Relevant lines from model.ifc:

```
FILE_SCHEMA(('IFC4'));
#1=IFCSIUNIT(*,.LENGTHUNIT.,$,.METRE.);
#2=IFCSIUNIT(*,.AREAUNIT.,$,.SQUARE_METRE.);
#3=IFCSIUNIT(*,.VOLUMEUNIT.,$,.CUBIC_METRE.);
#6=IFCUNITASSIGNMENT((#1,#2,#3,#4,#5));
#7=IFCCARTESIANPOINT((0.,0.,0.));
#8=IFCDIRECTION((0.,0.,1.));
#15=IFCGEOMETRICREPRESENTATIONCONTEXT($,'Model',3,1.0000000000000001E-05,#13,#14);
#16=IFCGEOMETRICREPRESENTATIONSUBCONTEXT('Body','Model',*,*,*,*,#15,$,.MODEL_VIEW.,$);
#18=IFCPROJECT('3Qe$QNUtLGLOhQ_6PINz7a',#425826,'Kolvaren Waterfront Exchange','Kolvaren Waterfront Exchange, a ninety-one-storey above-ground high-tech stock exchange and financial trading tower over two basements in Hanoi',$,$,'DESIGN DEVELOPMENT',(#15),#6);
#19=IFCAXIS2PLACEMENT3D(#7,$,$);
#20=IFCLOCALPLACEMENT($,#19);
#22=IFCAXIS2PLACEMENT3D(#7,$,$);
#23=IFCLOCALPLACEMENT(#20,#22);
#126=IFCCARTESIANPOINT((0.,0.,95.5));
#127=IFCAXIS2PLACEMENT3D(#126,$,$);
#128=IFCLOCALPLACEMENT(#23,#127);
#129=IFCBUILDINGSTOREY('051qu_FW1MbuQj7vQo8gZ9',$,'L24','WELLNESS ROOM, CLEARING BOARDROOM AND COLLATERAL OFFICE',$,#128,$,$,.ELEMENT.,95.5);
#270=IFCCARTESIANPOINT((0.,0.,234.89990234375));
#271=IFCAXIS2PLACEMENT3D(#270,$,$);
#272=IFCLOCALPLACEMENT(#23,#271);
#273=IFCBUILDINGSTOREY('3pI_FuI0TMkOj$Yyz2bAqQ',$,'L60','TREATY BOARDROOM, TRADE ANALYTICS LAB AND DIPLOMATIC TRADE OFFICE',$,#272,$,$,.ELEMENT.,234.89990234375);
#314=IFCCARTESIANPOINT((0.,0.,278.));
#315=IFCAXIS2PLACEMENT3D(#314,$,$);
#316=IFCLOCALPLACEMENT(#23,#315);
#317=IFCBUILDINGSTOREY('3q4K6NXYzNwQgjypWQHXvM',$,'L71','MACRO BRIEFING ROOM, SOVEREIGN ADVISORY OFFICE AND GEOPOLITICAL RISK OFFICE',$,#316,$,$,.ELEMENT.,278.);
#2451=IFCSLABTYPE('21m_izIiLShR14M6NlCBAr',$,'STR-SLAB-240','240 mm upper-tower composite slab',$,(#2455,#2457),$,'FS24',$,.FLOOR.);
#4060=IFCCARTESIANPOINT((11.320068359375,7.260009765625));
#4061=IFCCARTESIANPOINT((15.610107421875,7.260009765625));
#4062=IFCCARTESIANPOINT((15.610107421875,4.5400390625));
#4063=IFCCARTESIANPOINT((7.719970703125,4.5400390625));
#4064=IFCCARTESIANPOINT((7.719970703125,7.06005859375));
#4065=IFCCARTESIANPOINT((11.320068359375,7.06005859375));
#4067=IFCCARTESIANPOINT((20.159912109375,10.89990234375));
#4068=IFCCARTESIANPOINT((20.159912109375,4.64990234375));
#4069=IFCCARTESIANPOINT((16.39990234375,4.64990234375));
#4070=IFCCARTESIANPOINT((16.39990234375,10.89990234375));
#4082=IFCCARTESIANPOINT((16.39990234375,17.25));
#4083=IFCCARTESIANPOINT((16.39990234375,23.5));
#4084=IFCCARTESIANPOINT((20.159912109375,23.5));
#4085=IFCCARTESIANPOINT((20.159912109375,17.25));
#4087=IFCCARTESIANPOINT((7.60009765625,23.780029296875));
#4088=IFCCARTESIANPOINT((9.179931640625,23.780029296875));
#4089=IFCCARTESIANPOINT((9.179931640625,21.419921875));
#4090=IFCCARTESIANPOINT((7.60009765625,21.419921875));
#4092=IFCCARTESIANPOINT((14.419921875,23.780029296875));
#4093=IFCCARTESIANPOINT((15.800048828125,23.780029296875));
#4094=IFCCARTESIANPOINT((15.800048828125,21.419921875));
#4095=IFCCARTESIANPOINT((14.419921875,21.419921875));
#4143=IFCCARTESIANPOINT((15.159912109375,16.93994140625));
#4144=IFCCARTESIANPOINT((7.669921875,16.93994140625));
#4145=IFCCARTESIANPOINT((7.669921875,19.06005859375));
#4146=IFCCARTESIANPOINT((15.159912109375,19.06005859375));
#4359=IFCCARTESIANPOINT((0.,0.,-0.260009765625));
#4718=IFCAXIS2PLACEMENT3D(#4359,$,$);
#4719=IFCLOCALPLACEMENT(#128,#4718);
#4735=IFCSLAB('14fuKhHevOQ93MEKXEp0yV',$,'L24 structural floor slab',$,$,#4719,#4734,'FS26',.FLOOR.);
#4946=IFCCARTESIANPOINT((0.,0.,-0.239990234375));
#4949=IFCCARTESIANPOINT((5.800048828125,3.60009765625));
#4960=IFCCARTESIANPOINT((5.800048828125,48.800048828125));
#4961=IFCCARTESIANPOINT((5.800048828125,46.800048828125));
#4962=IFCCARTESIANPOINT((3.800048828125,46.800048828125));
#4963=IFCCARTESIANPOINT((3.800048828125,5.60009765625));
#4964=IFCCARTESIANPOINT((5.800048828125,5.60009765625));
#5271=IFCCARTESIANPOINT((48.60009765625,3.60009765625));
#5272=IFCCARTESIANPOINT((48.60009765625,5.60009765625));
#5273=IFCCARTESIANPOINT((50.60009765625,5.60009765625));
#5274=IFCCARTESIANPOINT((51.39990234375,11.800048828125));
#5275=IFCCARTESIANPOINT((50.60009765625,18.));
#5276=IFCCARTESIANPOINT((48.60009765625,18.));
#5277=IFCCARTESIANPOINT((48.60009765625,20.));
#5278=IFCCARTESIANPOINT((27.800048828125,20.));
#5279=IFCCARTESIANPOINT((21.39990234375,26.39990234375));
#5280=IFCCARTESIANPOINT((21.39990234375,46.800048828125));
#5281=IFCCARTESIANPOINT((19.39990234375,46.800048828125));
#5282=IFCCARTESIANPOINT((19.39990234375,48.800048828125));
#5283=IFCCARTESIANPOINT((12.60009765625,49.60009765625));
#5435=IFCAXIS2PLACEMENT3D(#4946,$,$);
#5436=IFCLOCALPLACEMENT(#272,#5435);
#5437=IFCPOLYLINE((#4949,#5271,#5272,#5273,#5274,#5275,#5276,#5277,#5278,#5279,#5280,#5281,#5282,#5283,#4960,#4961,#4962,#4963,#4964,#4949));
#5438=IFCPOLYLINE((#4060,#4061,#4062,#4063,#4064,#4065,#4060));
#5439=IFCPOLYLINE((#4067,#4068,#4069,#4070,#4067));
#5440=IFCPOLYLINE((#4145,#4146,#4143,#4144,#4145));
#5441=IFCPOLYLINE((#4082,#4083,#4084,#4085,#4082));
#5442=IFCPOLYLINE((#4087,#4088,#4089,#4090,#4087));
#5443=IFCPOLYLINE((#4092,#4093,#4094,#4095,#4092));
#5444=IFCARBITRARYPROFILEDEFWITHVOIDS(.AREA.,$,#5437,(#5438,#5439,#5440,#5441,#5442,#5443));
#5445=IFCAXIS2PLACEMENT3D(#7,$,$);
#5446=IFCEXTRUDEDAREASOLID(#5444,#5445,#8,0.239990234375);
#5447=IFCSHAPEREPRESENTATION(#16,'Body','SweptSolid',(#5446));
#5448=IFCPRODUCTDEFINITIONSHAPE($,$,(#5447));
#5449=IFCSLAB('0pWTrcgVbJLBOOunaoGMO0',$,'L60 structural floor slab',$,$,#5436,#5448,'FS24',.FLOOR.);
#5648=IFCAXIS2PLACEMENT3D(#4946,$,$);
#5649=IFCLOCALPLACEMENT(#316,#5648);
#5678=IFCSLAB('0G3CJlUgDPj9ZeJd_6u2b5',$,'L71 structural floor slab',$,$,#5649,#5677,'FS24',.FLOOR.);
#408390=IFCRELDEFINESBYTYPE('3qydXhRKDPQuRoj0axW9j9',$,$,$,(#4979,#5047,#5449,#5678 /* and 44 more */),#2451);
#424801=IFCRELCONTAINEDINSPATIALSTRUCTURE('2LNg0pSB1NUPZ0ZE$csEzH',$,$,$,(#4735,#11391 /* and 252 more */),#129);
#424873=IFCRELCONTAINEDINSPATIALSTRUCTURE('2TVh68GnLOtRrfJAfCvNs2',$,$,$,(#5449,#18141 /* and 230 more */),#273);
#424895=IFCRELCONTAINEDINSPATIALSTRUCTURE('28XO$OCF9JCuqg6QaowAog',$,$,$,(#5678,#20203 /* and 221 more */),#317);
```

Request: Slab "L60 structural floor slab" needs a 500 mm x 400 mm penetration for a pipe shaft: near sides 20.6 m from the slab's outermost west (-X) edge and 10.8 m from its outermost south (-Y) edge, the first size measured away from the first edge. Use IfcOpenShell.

```python
import numpy as np
import ifcopenshell
import ifcopenshell.api.feature
import ifcopenshell.api.geometry
import ifcopenshell.api.root
import ifcopenshell.geom
import ifcopenshell.util.placement
import ifcopenshell.util.representation
import ifcopenshell.util.shape
import ifcopenshell.util.unit

model = ifcopenshell.open("model.ifc")
unit_scale = ifcopenshell.util.unit.calculate_unit_scale(model)
settings = ifcopenshell.geom.settings()


def volume(element):
    """Net volume in cubic metres, openings subtracted."""
    shape = ifcopenshell.geom.create_shape(settings, element)
    return ifcopenshell.util.shape.get_volume(shape.geometry)


slab = model.by_guid("0pWTrcgVbJLBOOunaoGMO0")
before = volume(slab)

# Extent in the slab's own axes, in metres. The edges named are its -X and -Y sides.
slab_shape = ifcopenshell.geom.create_shape(settings, slab)
vertices = ifcopenshell.util.shape.get_vertices(slab_shape.geometry)
x_min, y_min, bottom = vertices.min(axis=0)
top = vertices[:, 2].max()

opening = ifcopenshell.api.root.create_entity(model, ifc_class="IfcOpeningElement", name="Pipe shaft opening", predefined_type="OPENING")
context = ifcopenshell.util.representation.get_context(model, "Model", "Body", "MODEL_VIEW")
width, depth = 0.5, 0.4
outline = [(0.0, 0.0), (width, 0.0), (width, depth), (0.0, depth), (0.0, 0.0)]
# Overshoot both faces by 50 mm so the cut is clean.
shape = ifcopenshell.api.geometry.add_slab_representation(
    model, context=context, depth=top - bottom + 0.1, polyline=outline
)
ifcopenshell.api.geometry.assign_representation(model, product=opening, representation=shape)

matrix = ifcopenshell.util.placement.get_local_placement(slab.ObjectPlacement)
matrix[:, 3] = matrix @ np.append(np.array([x_min + 20.6, y_min + 10.8, bottom - 0.05]) / unit_scale, 1.0)
ifcopenshell.api.geometry.edit_object_placement(model, product=opening, matrix=matrix, is_si=False)
ifcopenshell.api.feature.add_feature(model, feature=opening, element=slab)

after = volume(slab)

print(f"slab volume {before:.3f} -> {after:.3f} m3")

model.write("model_v2.ifc")
```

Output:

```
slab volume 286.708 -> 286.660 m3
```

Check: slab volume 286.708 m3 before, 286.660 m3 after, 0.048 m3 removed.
